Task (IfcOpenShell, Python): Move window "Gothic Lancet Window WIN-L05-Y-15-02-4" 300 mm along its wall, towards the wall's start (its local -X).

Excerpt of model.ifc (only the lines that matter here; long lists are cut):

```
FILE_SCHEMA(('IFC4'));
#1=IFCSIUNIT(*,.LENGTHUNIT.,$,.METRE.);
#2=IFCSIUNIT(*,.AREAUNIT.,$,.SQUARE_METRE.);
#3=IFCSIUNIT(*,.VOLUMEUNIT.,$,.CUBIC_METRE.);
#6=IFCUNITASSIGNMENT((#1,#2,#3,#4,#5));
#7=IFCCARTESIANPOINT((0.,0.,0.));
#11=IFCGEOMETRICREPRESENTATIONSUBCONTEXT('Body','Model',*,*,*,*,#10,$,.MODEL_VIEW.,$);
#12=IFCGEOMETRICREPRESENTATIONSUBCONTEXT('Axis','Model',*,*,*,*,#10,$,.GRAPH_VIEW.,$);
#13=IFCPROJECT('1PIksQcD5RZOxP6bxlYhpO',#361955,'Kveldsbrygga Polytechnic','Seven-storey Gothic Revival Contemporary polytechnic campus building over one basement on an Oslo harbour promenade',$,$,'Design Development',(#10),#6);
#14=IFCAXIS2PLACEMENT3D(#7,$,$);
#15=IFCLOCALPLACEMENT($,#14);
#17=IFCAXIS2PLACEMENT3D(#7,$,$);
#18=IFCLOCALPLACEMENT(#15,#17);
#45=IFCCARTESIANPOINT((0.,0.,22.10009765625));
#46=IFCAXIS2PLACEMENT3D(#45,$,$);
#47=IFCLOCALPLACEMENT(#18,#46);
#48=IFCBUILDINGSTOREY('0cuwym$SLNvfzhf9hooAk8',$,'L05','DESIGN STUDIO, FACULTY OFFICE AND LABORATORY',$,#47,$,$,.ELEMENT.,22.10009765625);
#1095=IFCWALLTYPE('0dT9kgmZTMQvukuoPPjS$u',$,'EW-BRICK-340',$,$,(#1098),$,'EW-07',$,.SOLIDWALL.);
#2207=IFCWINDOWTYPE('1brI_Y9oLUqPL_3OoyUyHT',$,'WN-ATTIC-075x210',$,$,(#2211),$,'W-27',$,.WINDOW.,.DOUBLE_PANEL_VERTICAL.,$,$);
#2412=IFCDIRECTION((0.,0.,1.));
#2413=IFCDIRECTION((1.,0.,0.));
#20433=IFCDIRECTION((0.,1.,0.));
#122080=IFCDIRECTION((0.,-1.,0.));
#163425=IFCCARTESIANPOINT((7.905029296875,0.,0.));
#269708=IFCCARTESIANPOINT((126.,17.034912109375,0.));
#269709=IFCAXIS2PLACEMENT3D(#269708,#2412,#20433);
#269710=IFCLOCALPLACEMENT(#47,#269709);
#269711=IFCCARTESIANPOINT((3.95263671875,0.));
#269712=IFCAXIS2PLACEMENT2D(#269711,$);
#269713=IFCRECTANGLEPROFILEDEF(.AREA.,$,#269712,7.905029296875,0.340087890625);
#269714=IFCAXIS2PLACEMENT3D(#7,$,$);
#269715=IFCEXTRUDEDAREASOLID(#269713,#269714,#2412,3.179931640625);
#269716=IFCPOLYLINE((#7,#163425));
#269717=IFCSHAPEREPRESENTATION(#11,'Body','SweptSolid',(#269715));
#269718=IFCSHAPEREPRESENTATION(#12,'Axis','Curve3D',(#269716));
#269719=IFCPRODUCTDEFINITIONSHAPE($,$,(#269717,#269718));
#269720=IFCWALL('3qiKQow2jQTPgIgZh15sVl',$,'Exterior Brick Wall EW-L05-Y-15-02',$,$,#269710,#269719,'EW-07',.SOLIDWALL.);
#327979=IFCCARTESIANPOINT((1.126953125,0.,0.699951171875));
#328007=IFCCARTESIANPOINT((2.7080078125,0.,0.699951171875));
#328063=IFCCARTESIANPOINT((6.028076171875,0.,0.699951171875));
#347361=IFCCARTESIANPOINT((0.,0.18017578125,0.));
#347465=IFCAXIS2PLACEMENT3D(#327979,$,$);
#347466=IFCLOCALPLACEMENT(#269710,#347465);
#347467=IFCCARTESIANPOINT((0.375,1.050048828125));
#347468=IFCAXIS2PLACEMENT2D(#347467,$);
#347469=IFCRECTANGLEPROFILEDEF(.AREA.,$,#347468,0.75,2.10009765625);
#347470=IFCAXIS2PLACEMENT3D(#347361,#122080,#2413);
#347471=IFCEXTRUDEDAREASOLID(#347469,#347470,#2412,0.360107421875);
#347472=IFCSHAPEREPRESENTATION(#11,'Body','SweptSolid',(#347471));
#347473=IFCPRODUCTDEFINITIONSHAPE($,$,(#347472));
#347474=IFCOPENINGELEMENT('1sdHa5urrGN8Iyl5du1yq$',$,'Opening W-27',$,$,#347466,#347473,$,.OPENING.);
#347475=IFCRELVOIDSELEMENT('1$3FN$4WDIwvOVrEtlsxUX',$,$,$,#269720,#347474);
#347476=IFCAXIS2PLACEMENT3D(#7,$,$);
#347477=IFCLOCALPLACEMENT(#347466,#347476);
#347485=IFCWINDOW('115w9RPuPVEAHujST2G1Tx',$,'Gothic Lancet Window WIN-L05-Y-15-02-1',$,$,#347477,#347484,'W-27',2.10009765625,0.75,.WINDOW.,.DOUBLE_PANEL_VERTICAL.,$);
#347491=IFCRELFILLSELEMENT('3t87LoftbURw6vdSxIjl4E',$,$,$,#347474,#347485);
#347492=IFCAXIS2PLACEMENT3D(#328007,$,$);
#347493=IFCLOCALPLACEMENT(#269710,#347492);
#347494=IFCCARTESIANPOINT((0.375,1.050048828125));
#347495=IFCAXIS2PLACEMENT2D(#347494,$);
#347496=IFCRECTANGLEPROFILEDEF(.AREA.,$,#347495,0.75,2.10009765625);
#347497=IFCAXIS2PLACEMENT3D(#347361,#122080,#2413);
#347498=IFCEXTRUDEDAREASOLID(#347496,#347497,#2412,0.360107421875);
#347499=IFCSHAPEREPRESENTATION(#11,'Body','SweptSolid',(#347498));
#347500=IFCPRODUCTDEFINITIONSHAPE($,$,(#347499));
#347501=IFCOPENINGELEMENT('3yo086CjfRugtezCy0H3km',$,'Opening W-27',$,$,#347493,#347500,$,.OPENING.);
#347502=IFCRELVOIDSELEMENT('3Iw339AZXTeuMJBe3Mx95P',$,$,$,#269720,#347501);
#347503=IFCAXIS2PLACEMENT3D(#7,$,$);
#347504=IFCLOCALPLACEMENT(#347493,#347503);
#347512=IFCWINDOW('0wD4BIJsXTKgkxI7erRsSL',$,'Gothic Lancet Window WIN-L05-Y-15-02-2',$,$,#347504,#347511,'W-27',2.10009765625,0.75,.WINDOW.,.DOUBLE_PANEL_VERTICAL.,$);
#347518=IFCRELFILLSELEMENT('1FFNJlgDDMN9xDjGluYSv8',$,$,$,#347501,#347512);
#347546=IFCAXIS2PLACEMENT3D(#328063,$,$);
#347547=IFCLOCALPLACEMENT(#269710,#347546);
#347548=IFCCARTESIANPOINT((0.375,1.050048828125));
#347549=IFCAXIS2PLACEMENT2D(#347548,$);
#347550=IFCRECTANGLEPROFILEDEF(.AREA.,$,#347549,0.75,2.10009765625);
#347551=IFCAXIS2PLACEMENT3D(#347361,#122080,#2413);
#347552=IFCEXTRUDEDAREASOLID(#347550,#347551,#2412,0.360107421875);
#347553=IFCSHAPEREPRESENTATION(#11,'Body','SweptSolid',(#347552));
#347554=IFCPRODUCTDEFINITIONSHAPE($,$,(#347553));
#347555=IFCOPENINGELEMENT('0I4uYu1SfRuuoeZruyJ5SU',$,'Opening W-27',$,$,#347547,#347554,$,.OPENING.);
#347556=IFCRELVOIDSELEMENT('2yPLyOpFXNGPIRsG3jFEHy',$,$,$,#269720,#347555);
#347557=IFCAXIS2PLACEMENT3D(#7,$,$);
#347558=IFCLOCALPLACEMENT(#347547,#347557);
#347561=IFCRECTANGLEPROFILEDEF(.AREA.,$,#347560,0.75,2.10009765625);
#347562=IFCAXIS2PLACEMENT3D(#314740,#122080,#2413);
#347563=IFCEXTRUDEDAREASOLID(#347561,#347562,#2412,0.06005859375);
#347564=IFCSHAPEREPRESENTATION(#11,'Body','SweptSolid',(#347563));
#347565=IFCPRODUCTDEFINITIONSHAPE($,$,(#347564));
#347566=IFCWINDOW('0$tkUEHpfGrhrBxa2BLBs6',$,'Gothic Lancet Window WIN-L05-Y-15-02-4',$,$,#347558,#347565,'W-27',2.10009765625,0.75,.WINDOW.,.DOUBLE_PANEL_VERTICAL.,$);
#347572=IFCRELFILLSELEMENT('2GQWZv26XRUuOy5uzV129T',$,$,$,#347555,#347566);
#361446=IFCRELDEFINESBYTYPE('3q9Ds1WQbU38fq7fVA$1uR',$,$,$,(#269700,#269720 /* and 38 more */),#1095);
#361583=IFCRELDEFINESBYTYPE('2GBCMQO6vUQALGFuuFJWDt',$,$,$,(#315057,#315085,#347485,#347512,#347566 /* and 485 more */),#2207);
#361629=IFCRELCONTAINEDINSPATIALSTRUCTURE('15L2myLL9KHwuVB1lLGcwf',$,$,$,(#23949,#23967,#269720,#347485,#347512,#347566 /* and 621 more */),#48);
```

```python
import ifcopenshell
import ifcopenshell.api.geometry
import ifcopenshell.util.placement

model = ifcopenshell.open("model.ifc")

window = model.by_guid("0$tkUEHpfGrhrBxa2BLBs6")
opening = window.FillsVoids[0].RelatingOpeningElement
wall = opening.VoidsElements[0].RelatingBuildingElement

wall_matrix = ifcopenshell.util.placement.get_local_placement(wall.ObjectPlacement)
shift = wall_matrix[:3, 0] * -0.3
before = ifcopenshell.util.placement.get_local_placement(window.ObjectPlacement)[:3, 3].copy()

# The window is placed relative to its opening, so it follows when the opening moves.
matrix = ifcopenshell.util.placement.get_local_placement(opening.ObjectPlacement)
matrix[:3, 3] += shift
ifcopenshell.api.geometry.edit_object_placement(
    model, product=opening, matrix=matrix, is_si=False, should_transform_children=True
)

after = ifcopenshell.util.placement.get_local_placement(window.ObjectPlacement)[:3, 3]
print("window moved by", (after - before).round(3) + 0.0)

model.write("model_edited.ifc")
```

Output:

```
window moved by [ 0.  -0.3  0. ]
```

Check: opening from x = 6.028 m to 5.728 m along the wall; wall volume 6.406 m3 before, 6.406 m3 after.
